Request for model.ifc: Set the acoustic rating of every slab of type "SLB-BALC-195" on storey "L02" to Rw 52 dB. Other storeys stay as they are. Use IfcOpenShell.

First a look at what the model holds.

```python
import ifcopenshell
import ifcopenshell.util.element

model = ifcopenshell.open("model.ifc")
print(model.schema)
storey = next(s for s in model.by_type("IfcBuildingStorey") if s.Name == "L02")
slabs = [e for e in ifcopenshell.util.element.get_decomposition(storey) if e.is_a("IfcSlab")]
seen = {}
for e in slabs:
    element_type = ifcopenshell.util.element.get_type(e)
    key = (element_type.Name if element_type != e and element_type else None, ifcopenshell.util.element.get_pset(e, "Pset_SlabCommon", "AcousticRating"))
    seen[key] = seen.get(key, 0) + 1
for (name, value), count in sorted(seen.items(), key=str):
    print(count, "x", name, "|", value)
```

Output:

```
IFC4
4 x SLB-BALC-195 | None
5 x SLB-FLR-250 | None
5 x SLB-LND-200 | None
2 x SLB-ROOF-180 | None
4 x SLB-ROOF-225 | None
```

```python
import ifcopenshell
import ifcopenshell.api.pset
import ifcopenshell.util.element

model = ifcopenshell.open("model.ifc")

storey = next(s for s in model.by_type("IfcBuildingStorey") if s.Name == "L02")
slabs = [e for e in ifcopenshell.util.element.get_decomposition(storey) if e.is_a("IfcSlab")]

count = 0
for e in slabs:
    element_type = ifcopenshell.util.element.get_type(e)
    if element_type in (None, e) or element_type.Name != "SLB-BALC-195":
        continue
    # add_pset returns the element's existing set when there is one.
    pset = ifcopenshell.api.pset.add_pset(model, product=e, name="Pset_SlabCommon")
    ifcopenshell.api.pset.edit_pset(model, pset=pset, properties={"AcousticRating": "Rw 52 dB"})
    count += 1

print(count, "slabs updated")

model.write("model_edited.ifc")
```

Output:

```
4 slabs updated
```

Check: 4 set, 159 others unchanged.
